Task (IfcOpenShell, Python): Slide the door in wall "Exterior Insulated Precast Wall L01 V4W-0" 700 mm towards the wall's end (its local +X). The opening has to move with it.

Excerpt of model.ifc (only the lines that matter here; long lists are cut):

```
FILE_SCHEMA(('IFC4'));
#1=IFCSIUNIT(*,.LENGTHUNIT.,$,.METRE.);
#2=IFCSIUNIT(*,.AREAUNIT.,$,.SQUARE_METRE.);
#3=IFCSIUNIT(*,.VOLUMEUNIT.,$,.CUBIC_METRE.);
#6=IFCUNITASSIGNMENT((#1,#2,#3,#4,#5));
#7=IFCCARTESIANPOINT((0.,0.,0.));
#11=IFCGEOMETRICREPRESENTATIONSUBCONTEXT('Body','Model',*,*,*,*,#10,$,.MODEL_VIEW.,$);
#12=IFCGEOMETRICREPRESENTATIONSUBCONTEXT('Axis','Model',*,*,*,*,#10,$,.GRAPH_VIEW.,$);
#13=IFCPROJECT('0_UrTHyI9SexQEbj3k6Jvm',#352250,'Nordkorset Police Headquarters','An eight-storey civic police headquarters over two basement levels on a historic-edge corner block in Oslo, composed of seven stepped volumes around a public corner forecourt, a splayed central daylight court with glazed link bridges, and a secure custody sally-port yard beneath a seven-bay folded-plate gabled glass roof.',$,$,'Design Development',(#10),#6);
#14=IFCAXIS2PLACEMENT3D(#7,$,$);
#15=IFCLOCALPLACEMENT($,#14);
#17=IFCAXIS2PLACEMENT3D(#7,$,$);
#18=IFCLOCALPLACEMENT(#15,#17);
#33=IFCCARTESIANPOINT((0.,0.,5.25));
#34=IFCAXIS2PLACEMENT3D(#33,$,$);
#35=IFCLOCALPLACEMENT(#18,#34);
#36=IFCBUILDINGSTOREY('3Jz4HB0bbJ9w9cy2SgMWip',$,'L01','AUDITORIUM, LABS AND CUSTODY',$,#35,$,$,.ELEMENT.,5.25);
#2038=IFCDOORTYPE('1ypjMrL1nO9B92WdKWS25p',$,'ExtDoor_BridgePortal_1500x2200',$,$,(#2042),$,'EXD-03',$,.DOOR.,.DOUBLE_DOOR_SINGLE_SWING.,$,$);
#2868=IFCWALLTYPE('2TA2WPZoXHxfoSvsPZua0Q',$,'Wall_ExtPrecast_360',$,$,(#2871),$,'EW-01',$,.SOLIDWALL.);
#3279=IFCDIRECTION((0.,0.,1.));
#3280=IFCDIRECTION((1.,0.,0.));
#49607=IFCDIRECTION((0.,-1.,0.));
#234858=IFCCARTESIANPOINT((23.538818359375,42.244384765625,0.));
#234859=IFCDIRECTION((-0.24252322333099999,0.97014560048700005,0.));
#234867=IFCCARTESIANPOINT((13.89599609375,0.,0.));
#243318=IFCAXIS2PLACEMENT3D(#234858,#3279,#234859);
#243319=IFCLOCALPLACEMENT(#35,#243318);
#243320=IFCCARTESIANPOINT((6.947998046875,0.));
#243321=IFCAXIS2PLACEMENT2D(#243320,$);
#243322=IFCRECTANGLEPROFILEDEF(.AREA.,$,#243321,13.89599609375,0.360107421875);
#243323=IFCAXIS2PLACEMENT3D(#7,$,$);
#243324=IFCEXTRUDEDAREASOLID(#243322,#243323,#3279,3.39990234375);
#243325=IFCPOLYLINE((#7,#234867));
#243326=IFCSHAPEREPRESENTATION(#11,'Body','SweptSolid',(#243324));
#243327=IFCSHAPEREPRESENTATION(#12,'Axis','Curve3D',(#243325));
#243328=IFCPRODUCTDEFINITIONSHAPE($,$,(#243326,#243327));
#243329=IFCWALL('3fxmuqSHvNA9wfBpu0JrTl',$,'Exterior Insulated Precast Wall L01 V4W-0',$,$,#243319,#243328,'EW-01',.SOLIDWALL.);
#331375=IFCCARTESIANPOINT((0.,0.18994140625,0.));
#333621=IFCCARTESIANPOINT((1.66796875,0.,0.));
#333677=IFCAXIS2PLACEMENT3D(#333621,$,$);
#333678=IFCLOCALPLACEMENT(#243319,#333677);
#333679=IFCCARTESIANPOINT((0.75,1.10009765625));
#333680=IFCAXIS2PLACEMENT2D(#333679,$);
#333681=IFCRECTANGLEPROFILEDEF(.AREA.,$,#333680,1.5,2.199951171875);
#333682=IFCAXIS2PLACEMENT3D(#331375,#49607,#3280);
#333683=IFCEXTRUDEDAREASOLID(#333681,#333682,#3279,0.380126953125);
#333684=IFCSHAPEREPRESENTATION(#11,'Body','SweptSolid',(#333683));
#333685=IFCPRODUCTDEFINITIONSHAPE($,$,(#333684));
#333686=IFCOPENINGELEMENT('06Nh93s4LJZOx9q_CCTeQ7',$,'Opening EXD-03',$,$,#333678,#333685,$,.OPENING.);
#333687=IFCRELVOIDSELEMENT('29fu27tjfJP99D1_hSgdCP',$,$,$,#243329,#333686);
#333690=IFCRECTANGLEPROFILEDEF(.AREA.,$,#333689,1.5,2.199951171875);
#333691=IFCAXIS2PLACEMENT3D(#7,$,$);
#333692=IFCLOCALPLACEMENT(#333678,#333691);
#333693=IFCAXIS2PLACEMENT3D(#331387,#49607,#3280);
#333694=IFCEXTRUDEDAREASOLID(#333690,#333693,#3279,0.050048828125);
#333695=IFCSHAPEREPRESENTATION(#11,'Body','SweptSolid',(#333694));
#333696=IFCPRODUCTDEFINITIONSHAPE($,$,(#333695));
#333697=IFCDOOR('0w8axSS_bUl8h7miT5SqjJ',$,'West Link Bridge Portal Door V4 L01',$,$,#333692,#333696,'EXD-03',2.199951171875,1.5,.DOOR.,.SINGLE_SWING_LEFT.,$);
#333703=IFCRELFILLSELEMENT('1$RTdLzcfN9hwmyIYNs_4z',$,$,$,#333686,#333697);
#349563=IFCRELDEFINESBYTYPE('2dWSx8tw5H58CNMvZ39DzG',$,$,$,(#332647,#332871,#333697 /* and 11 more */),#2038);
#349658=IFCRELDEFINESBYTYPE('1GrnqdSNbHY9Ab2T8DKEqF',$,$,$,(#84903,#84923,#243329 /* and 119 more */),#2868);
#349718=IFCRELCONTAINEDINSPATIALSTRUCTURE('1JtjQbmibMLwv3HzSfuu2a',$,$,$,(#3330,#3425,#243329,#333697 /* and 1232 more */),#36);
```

```python
import ifcopenshell
import ifcopenshell.api.geometry
import ifcopenshell.util.placement
import ifcopenshell.util.unit

model = ifcopenshell.open("model.ifc")
unit_scale = ifcopenshell.util.unit.calculate_unit_scale(model)

door = model.by_guid("0w8axSS_bUl8h7miT5SqjJ")
opening = door.FillsVoids[0].RelatingOpeningElement
wall = opening.VoidsElements[0].RelatingBuildingElement

wall_matrix = ifcopenshell.util.placement.get_local_placement(wall.ObjectPlacement)
shift = wall_matrix[:3, 0] * 0.7 / unit_scale
before = ifcopenshell.util.placement.get_local_placement(door.ObjectPlacement)[:3, 3].copy()

# The door is placed relative to its opening, so it follows when the opening moves.
matrix = ifcopenshell.util.placement.get_local_placement(opening.ObjectPlacement)
matrix[:3, 3] += shift
ifcopenshell.api.geometry.edit_object_placement(
    model, product=opening, matrix=matrix, is_si=False, should_transform_children=True
)

after = ifcopenshell.util.placement.get_local_placement(door.ObjectPlacement)[:3, 3]
print("door moved by", (after - before).round(3) + 0.0)

model.write("model_v2.ifc")
```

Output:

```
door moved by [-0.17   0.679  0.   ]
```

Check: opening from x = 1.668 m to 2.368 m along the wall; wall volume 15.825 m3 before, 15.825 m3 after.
